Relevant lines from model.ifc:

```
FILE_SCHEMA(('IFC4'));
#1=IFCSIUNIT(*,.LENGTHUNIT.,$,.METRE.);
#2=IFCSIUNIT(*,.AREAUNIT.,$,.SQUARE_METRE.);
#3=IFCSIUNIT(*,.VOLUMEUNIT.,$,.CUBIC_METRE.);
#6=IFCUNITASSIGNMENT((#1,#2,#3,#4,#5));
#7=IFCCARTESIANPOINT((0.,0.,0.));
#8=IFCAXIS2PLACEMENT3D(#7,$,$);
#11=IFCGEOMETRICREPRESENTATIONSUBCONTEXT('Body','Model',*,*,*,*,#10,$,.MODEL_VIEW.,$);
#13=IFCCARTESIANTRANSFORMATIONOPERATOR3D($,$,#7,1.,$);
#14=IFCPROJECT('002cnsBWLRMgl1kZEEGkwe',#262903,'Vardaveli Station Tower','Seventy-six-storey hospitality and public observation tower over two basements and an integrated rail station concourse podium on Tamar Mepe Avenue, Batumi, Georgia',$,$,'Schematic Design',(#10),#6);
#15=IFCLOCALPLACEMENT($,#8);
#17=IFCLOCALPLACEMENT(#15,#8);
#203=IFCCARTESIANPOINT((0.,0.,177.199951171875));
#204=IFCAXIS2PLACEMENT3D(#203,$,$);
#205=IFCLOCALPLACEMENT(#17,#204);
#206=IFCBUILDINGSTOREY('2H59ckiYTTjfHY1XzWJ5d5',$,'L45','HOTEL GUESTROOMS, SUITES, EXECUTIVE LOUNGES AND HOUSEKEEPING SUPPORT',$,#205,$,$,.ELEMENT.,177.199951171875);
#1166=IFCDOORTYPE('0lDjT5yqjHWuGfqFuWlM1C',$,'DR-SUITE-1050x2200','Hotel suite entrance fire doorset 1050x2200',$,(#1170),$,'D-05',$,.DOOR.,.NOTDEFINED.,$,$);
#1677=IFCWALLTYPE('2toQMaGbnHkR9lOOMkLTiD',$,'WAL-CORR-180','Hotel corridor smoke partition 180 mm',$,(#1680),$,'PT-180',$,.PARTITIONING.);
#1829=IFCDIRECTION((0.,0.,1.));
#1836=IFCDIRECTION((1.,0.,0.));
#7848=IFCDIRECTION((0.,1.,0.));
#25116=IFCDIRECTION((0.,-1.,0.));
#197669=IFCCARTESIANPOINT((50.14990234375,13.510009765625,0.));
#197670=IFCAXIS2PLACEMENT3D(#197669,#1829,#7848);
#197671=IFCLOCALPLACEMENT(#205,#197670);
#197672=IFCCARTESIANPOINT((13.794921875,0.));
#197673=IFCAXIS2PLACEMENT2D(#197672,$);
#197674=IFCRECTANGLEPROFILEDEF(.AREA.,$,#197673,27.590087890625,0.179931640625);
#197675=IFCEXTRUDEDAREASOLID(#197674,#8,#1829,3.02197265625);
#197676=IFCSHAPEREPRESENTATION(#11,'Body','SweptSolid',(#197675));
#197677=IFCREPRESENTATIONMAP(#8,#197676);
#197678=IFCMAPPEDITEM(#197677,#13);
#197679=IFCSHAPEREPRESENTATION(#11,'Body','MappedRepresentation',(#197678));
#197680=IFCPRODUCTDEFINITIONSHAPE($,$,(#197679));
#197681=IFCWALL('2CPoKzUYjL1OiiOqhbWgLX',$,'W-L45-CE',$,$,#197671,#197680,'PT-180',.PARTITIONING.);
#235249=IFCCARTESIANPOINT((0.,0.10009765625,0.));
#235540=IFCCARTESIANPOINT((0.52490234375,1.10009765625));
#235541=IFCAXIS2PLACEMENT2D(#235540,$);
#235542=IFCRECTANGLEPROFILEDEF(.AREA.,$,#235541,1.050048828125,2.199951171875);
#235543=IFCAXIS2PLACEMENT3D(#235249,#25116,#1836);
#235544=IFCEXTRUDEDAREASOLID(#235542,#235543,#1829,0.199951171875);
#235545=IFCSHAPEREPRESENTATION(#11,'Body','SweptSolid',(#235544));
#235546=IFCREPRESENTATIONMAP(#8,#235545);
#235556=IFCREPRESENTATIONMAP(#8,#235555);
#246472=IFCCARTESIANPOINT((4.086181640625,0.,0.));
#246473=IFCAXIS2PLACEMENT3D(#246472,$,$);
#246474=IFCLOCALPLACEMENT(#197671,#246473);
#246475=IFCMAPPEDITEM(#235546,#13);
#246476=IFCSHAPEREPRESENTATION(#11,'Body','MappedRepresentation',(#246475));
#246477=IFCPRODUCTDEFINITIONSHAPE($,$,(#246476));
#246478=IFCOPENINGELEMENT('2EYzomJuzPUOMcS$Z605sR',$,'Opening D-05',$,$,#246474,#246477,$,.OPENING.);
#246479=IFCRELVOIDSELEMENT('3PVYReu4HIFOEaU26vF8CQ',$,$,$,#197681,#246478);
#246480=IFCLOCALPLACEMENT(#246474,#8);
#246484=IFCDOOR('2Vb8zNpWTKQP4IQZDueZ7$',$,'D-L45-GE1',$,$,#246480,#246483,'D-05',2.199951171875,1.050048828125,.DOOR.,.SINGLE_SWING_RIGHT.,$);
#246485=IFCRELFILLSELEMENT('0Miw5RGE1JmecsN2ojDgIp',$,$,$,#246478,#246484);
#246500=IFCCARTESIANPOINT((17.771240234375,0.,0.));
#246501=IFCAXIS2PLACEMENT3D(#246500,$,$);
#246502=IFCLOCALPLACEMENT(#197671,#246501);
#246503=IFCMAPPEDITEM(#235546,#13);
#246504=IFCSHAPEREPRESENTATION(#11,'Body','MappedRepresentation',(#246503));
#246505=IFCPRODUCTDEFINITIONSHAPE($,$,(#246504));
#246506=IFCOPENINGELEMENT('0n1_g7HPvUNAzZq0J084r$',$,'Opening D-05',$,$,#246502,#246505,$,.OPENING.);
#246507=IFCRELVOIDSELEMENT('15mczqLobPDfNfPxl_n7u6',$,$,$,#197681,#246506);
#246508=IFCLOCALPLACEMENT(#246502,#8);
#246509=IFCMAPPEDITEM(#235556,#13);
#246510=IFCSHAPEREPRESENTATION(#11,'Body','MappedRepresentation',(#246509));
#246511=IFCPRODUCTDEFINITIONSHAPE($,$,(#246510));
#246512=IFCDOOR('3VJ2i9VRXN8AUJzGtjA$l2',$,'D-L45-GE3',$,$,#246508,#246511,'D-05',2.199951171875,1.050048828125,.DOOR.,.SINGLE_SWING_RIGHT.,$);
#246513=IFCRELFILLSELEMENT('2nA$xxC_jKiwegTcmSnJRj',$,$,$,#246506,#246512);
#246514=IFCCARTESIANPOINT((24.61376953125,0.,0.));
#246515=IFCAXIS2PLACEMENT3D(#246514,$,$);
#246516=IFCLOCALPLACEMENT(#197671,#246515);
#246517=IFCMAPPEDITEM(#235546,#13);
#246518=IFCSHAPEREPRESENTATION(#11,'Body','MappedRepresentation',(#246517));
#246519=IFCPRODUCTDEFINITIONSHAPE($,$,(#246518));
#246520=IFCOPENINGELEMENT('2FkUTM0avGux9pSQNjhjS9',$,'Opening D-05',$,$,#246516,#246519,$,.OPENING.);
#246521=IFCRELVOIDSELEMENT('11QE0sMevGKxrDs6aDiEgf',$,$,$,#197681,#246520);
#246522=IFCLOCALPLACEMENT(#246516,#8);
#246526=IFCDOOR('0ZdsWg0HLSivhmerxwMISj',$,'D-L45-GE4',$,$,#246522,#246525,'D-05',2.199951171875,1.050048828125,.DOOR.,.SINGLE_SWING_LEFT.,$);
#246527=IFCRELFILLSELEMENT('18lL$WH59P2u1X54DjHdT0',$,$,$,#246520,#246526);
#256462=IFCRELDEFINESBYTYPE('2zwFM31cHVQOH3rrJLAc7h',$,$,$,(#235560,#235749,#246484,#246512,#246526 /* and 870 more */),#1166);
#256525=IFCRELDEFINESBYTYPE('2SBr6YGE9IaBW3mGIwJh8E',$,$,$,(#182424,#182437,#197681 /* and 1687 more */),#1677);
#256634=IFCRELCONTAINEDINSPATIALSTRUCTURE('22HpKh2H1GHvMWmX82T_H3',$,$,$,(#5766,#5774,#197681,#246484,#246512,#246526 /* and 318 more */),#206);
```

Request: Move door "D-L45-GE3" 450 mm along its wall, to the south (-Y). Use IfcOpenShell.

```python
import ifcopenshell
import ifcopenshell.api.geometry
import ifcopenshell.util.placement
import ifcopenshell.util.unit

model = ifcopenshell.open("model.ifc")
unit_scale = ifcopenshell.util.unit.calculate_unit_scale(model)

door = model.by_guid("3VJ2i9VRXN8AUJzGtjA$l2")
opening = door.FillsVoids[0].RelatingOpeningElement
wall = opening.VoidsElements[0].RelatingBuildingElement

wall_matrix = ifcopenshell.util.placement.get_local_placement(wall.ObjectPlacement)
shift = wall_matrix[:3, 0] * -0.45 / unit_scale
before = ifcopenshell.util.placement.get_local_placement(door.ObjectPlacement)[:3, 3].copy()

# The door is placed relative to its opening, so it follows when the opening moves.
matrix = ifcopenshell.util.placement.get_local_placement(opening.ObjectPlacement)
matrix[:3, 3] += shift
ifcopenshell.api.geometry.edit_object_placement(
    model, product=opening, matrix=matrix, is_si=False, should_transform_children=True
)

after = ifcopenshell.util.placement.get_local_placement(door.ObjectPlacement)[:3, 3]
print("door moved by", (after - before).round(3) + 0.0)

model.write("model_rev.ifc")
```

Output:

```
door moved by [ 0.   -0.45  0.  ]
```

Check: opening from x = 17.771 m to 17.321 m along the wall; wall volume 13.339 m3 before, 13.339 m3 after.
